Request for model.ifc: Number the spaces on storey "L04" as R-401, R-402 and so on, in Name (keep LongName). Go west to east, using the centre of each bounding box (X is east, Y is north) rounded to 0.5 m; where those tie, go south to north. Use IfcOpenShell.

First a look at what the model holds.

```python
import ifcopenshell
import ifcopenshell.util.element
import ifcopenshell.util.placement

model = ifcopenshell.open("model.ifc")
print(model.schema)
storey = next(s for s in model.by_type("IfcBuildingStorey") if s.Name == "L04")
spaces = [e for e in ifcopenshell.util.element.get_decomposition(storey) if e.is_a("IfcSpace")]
for e in sorted(spaces, key=lambda e: e.id()):
    origin = ifcopenshell.util.placement.get_local_placement(e.ObjectPlacement)[:3, 3]
    print(e.id(), e.Name, e.LongName, origin.round(2) + 0.0, sep=" | ")
```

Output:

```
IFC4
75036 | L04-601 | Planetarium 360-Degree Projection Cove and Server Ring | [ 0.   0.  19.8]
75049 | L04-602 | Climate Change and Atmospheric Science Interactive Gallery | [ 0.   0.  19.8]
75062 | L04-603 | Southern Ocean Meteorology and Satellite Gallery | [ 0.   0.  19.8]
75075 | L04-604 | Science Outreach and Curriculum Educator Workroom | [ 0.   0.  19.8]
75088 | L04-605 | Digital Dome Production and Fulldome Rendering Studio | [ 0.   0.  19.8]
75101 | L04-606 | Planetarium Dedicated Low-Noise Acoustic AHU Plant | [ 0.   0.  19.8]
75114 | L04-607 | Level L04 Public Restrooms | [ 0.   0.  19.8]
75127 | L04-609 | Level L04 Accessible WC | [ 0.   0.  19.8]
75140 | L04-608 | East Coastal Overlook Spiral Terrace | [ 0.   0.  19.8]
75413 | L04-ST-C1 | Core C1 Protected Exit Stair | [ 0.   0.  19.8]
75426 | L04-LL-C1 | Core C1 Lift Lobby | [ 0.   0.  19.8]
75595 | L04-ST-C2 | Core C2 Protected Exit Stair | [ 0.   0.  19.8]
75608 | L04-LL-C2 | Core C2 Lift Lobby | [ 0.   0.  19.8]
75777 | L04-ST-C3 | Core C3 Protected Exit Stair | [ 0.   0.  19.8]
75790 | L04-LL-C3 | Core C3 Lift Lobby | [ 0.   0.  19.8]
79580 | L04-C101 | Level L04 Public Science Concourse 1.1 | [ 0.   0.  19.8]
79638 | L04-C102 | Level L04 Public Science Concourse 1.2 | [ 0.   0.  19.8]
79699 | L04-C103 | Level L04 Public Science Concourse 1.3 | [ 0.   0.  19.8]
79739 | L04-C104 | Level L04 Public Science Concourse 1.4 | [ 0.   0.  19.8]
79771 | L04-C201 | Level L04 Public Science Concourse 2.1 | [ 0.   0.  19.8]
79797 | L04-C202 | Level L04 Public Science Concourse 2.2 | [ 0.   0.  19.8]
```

```python
import ifcopenshell
import ifcopenshell.geom
import ifcopenshell.util.element
import ifcopenshell.util.shape

model = ifcopenshell.open("model.ifc")
settings = ifcopenshell.geom.settings()
settings.set("use-world-coords", True)


def centre(element):
    shape = ifcopenshell.geom.create_shape(settings, element)
    return ifcopenshell.util.shape.get_bbox_centroid(shape.geometry)


storey = next(s for s in model.by_type("IfcBuildingStorey") if s.Name == "L04")
spaces = [e for e in ifcopenshell.util.element.get_decomposition(storey) if e.is_a("IfcSpace")]

# Insertion points can sit at a corner or the storey origin, so sort by the geometry (in metres).
centres = {e: centre(e) for e in spaces}
spaces.sort(key=lambda e: (round(centres[e][0] / 0.5), centres[e][1]))

for i, e in enumerate(spaces, start=1):
    number = f"R-4{i:02d}"
    e.Name = number
    print(e.id(), number)

model.write("model_updated.ifc")
```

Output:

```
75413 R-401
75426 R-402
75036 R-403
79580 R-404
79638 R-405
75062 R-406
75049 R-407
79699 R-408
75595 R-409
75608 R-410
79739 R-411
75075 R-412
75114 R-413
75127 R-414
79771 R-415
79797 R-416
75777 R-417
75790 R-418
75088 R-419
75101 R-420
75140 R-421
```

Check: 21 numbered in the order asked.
